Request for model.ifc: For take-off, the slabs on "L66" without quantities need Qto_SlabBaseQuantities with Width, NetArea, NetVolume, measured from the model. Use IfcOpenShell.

First a look at what the model holds.

```python
import ifcopenshell
import ifcopenshell.util.element
import ifcopenshell.util.unit

model = ifcopenshell.open("model.ifc")
print(model.schema)
for unit_type in ("LENGTHUNIT", "AREAUNIT", "VOLUMEUNIT"):
    print(unit_type, ifcopenshell.util.unit.calculate_unit_scale(model, unit_type))
storey = next(s for s in model.by_type("IfcBuildingStorey") if s.Name == "L66")
slabs = [e for e in ifcopenshell.util.element.get_decomposition(storey) if e.is_a("IfcSlab")]
for e in sorted(slabs, key=lambda e: e.id()):
    print(e.id(), e.is_a(), e.Name, list(ifcopenshell.util.element.get_psets(e, qtos_only=True)), sep=" | ")
```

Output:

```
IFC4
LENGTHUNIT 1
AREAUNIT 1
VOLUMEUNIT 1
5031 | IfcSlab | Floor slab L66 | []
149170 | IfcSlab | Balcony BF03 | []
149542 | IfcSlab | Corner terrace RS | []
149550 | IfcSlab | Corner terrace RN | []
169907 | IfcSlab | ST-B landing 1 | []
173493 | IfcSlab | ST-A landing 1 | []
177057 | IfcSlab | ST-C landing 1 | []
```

```python
import ifcopenshell
import ifcopenshell.api.pset
import ifcopenshell.geom
import ifcopenshell.util.element
import ifcopenshell.util.shape
import ifcopenshell.util.unit

model = ifcopenshell.open("model.ifc")
unit_scale = ifcopenshell.util.unit.calculate_unit_scale(model)
area_scale = ifcopenshell.util.unit.calculate_unit_scale(model, "AREAUNIT")
volume_scale = ifcopenshell.util.unit.calculate_unit_scale(model, "VOLUMEUNIT")
settings = ifcopenshell.geom.settings()

storey = next(s for s in model.by_type("IfcBuildingStorey") if s.Name == "L66")
slabs = [e for e in ifcopenshell.util.element.get_decomposition(storey) if e.is_a("IfcSlab")]

for e in sorted(slabs, key=lambda e: e.id()):
    if ifcopenshell.util.element.get_psets(e, qtos_only=True, should_inherit=False):
        continue
    # Geometry comes back in metres, in the element's own axes.
    shape = ifcopenshell.geom.create_shape(settings, e)
    values = {
        "Width": ifcopenshell.util.shape.get_z(shape.geometry) / unit_scale,
        "NetArea": ifcopenshell.util.shape.get_footprint_area(shape.geometry) / area_scale,
        "NetVolume": ifcopenshell.util.shape.get_volume(shape.geometry) / volume_scale,
    }
    qto = ifcopenshell.api.pset.add_qto(model, product=e, name="Qto_SlabBaseQuantities")
    ifcopenshell.api.pset.edit_qto(model, qto=qto, properties=values)
    print(e.id(), {k: round(v, 3) for k, v in values.items()})

model.write("model-out.ifc")
```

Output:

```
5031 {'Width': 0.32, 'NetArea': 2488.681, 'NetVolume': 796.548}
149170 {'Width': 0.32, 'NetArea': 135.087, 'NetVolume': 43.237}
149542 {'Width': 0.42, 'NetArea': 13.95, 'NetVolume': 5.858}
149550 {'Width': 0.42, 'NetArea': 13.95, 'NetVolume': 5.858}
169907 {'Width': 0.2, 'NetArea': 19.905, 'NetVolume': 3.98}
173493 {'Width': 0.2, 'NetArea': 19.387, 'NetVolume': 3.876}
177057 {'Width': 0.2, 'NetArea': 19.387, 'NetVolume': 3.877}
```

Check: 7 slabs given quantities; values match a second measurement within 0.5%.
